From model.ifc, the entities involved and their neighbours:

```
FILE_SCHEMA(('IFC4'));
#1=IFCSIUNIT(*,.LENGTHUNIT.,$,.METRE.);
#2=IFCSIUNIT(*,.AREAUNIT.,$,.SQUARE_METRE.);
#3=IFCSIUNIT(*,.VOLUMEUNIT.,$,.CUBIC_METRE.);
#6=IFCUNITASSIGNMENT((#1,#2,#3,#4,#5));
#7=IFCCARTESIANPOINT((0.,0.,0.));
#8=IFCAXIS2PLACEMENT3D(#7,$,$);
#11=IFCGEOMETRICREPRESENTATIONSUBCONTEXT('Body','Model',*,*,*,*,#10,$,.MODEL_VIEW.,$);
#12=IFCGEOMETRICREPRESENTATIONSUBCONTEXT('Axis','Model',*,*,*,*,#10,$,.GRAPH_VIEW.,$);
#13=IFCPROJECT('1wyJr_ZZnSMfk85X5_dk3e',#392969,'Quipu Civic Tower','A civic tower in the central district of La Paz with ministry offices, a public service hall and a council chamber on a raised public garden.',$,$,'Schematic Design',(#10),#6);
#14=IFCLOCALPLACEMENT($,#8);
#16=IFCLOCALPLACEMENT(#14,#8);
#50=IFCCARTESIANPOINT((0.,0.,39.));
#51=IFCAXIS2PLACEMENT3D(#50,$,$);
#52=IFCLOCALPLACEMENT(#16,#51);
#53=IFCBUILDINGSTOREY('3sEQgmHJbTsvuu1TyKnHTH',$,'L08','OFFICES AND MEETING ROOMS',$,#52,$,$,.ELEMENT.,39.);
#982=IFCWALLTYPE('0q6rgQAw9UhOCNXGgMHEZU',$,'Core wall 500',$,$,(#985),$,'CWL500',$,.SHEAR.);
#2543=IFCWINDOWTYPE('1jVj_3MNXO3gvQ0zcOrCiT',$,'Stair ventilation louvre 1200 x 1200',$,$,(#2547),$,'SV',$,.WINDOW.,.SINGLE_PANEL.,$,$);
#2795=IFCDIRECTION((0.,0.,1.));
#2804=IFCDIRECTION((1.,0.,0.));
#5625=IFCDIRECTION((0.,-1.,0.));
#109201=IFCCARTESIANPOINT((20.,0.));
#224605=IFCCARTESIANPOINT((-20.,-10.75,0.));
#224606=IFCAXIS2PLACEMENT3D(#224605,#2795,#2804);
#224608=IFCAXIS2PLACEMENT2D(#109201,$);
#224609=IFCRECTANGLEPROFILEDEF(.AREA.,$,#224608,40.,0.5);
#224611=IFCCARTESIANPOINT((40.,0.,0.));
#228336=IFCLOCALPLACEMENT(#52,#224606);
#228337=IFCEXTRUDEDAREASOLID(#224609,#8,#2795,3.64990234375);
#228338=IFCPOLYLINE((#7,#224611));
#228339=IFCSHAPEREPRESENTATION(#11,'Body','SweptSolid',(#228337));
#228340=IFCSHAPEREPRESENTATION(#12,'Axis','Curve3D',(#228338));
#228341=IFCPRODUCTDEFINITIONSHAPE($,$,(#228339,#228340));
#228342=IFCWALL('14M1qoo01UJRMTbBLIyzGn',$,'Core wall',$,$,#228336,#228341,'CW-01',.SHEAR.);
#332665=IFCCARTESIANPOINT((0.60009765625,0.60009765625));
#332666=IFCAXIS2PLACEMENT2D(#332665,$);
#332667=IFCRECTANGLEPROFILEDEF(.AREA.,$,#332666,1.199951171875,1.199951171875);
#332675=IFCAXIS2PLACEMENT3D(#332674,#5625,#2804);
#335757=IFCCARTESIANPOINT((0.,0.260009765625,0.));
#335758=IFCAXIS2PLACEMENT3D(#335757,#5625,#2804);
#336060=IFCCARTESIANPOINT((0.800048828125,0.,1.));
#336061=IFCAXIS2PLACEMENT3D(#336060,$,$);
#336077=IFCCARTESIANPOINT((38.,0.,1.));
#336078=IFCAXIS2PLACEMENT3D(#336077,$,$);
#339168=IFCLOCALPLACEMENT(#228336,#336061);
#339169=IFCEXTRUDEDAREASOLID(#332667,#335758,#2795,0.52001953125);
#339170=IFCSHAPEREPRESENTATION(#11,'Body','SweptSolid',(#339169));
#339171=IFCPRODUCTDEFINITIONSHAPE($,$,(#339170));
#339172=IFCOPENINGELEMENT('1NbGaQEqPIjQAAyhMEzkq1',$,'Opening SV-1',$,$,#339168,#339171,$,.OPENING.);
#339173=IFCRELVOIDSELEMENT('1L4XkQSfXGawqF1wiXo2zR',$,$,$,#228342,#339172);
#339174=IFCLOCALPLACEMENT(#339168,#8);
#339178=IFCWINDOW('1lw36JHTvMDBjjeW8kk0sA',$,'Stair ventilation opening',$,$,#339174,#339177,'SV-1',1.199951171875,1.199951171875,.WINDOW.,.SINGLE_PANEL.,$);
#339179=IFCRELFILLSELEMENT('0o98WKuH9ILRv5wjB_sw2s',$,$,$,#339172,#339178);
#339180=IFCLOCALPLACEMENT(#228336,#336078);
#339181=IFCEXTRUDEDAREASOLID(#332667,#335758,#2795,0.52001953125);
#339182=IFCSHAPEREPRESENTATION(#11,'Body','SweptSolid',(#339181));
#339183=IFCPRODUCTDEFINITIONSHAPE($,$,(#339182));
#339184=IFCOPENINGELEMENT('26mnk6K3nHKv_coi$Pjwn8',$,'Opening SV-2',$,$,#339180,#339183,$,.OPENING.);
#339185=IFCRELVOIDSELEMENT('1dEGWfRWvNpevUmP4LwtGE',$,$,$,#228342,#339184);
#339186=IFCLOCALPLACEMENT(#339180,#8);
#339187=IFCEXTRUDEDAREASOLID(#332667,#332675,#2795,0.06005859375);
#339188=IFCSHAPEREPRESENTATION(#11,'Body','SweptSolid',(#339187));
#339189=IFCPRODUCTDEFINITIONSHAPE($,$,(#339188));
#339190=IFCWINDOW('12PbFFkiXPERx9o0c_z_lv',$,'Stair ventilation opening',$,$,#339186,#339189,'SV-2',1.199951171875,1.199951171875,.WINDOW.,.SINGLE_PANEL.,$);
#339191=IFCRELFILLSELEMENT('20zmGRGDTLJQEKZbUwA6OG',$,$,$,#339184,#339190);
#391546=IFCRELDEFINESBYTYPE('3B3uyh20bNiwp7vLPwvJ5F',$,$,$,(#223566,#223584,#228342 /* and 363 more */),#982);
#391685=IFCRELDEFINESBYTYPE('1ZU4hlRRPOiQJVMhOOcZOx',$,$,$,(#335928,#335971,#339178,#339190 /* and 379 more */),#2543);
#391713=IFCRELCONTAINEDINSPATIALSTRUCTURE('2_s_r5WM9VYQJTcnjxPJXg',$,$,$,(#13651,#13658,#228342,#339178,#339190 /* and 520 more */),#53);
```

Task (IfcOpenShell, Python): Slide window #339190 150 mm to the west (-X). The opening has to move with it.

```python
import ifcopenshell
import ifcopenshell.api.geometry
import ifcopenshell.util.placement

model = ifcopenshell.open("model.ifc")

window = model.by_guid("12PbFFkiXPERx9o0c_z_lv")
opening = window.FillsVoids[0].RelatingOpeningElement
wall = opening.VoidsElements[0].RelatingBuildingElement

wall_matrix = ifcopenshell.util.placement.get_local_placement(wall.ObjectPlacement)
shift = wall_matrix[:3, 0] * -0.15
before = ifcopenshell.util.placement.get_local_placement(window.ObjectPlacement)[:3, 3].copy()

# The window is placed relative to its opening, so it follows when the opening moves.
matrix = ifcopenshell.util.placement.get_local_placement(opening.ObjectPlacement)
matrix[:3, 3] += shift
ifcopenshell.api.geometry.edit_object_placement(
    model, product=opening, matrix=matrix, is_si=False, should_transform_children=True
)

after = ifcopenshell.util.placement.get_local_placement(window.ObjectPlacement)[:3, 3]
print("window moved by", (after - before).round(3) + 0.0)

model.write("model_rev.ifc")
```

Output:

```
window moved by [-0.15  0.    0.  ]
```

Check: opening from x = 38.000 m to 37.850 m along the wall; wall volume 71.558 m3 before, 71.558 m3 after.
